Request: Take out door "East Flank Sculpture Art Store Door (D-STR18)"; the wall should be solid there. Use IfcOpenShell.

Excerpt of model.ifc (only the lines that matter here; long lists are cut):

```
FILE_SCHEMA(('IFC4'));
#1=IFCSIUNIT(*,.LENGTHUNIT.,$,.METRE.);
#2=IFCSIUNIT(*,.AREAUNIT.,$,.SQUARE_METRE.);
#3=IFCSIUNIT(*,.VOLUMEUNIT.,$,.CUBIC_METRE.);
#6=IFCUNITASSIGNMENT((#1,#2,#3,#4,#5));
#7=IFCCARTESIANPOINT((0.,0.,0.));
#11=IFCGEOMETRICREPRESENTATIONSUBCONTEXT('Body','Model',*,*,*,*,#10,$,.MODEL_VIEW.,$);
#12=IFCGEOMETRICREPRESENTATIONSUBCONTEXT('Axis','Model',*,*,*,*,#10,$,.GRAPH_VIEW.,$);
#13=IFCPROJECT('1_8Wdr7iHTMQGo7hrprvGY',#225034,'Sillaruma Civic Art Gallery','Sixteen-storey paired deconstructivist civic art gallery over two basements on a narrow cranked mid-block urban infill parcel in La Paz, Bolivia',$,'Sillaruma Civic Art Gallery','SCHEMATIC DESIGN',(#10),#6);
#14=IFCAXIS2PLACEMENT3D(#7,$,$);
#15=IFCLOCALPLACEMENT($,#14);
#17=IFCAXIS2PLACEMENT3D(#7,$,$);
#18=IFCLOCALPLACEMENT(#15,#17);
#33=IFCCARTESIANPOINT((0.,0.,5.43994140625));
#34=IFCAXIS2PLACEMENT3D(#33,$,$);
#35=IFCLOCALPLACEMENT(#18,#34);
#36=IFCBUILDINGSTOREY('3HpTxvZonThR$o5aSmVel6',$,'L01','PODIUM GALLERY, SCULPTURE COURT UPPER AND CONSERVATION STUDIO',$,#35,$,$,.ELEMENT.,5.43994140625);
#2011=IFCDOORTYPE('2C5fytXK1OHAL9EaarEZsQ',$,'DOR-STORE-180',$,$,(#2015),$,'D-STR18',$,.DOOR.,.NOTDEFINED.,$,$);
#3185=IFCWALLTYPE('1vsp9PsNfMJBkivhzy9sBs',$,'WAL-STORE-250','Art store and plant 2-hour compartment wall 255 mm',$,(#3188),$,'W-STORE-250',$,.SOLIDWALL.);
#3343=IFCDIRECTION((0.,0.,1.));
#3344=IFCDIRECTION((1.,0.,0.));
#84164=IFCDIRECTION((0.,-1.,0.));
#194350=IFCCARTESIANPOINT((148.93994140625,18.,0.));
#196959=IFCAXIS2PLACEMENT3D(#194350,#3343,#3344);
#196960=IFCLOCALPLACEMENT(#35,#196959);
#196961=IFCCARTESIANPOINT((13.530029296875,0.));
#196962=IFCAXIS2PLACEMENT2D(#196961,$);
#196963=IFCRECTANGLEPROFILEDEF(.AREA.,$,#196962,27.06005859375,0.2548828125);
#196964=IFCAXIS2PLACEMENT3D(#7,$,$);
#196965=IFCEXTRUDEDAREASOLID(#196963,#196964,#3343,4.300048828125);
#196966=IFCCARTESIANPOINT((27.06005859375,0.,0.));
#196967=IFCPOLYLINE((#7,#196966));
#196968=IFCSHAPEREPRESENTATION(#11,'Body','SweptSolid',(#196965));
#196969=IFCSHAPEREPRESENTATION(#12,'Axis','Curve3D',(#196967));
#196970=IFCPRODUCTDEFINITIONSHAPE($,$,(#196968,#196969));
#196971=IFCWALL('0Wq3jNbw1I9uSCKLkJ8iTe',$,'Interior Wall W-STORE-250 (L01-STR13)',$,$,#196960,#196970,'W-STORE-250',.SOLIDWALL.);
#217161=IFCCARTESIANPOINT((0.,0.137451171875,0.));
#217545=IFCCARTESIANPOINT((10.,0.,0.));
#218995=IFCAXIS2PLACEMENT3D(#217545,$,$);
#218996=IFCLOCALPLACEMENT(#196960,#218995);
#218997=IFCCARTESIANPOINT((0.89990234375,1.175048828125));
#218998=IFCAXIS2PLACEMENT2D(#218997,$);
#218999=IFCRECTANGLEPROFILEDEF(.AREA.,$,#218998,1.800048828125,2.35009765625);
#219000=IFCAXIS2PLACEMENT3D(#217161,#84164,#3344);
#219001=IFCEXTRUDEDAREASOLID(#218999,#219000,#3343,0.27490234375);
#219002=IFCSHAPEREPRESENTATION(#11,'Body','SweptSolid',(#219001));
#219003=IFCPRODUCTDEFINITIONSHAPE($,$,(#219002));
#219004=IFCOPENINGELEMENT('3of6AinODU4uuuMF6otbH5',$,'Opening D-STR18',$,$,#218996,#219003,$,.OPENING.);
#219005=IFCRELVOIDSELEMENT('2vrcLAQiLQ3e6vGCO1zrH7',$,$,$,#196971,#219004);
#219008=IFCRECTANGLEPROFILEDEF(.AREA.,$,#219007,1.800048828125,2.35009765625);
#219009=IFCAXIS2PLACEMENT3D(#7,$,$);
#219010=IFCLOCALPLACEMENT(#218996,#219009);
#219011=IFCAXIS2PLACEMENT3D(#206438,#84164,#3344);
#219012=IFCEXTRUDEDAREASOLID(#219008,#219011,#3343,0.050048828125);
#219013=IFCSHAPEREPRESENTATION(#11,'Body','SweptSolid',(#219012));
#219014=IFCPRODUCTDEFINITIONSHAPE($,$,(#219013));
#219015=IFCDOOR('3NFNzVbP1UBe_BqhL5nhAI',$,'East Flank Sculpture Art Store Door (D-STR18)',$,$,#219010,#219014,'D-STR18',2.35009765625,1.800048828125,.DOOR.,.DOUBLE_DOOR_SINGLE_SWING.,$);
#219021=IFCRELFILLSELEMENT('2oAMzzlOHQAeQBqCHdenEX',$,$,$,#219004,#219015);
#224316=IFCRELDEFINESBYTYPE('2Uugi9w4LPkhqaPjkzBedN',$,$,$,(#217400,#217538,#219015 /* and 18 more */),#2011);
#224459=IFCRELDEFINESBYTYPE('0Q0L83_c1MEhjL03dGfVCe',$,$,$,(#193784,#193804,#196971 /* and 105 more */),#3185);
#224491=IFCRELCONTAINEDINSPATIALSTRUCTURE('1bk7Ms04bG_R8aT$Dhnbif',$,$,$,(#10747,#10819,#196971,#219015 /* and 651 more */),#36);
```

```python
import ifcopenshell
import ifcopenshell.api.feature
import ifcopenshell.api.root
import ifcopenshell.geom
import ifcopenshell.util.shape

model = ifcopenshell.open("model.ifc")
settings = ifcopenshell.geom.settings()


def volume(element):
    """Net volume in cubic metres, openings subtracted."""
    shape = ifcopenshell.geom.create_shape(settings, element)
    return ifcopenshell.util.shape.get_volume(shape.geometry)


door = model.by_id(219015)
opening = door.FillsVoids[0].RelatingOpeningElement
wall = opening.VoidsElements[0].RelatingBuildingElement
before = volume(wall)

ifcopenshell.api.root.remove_product(model, product=door)
ifcopenshell.api.feature.remove_feature(model, feature=opening)

after = volume(wall)

print(f"wall volume {before:.3f} -> {after:.3f} m3")

model.write("model_rev.ifc")
```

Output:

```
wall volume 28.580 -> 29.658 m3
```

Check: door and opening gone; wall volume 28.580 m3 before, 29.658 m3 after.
